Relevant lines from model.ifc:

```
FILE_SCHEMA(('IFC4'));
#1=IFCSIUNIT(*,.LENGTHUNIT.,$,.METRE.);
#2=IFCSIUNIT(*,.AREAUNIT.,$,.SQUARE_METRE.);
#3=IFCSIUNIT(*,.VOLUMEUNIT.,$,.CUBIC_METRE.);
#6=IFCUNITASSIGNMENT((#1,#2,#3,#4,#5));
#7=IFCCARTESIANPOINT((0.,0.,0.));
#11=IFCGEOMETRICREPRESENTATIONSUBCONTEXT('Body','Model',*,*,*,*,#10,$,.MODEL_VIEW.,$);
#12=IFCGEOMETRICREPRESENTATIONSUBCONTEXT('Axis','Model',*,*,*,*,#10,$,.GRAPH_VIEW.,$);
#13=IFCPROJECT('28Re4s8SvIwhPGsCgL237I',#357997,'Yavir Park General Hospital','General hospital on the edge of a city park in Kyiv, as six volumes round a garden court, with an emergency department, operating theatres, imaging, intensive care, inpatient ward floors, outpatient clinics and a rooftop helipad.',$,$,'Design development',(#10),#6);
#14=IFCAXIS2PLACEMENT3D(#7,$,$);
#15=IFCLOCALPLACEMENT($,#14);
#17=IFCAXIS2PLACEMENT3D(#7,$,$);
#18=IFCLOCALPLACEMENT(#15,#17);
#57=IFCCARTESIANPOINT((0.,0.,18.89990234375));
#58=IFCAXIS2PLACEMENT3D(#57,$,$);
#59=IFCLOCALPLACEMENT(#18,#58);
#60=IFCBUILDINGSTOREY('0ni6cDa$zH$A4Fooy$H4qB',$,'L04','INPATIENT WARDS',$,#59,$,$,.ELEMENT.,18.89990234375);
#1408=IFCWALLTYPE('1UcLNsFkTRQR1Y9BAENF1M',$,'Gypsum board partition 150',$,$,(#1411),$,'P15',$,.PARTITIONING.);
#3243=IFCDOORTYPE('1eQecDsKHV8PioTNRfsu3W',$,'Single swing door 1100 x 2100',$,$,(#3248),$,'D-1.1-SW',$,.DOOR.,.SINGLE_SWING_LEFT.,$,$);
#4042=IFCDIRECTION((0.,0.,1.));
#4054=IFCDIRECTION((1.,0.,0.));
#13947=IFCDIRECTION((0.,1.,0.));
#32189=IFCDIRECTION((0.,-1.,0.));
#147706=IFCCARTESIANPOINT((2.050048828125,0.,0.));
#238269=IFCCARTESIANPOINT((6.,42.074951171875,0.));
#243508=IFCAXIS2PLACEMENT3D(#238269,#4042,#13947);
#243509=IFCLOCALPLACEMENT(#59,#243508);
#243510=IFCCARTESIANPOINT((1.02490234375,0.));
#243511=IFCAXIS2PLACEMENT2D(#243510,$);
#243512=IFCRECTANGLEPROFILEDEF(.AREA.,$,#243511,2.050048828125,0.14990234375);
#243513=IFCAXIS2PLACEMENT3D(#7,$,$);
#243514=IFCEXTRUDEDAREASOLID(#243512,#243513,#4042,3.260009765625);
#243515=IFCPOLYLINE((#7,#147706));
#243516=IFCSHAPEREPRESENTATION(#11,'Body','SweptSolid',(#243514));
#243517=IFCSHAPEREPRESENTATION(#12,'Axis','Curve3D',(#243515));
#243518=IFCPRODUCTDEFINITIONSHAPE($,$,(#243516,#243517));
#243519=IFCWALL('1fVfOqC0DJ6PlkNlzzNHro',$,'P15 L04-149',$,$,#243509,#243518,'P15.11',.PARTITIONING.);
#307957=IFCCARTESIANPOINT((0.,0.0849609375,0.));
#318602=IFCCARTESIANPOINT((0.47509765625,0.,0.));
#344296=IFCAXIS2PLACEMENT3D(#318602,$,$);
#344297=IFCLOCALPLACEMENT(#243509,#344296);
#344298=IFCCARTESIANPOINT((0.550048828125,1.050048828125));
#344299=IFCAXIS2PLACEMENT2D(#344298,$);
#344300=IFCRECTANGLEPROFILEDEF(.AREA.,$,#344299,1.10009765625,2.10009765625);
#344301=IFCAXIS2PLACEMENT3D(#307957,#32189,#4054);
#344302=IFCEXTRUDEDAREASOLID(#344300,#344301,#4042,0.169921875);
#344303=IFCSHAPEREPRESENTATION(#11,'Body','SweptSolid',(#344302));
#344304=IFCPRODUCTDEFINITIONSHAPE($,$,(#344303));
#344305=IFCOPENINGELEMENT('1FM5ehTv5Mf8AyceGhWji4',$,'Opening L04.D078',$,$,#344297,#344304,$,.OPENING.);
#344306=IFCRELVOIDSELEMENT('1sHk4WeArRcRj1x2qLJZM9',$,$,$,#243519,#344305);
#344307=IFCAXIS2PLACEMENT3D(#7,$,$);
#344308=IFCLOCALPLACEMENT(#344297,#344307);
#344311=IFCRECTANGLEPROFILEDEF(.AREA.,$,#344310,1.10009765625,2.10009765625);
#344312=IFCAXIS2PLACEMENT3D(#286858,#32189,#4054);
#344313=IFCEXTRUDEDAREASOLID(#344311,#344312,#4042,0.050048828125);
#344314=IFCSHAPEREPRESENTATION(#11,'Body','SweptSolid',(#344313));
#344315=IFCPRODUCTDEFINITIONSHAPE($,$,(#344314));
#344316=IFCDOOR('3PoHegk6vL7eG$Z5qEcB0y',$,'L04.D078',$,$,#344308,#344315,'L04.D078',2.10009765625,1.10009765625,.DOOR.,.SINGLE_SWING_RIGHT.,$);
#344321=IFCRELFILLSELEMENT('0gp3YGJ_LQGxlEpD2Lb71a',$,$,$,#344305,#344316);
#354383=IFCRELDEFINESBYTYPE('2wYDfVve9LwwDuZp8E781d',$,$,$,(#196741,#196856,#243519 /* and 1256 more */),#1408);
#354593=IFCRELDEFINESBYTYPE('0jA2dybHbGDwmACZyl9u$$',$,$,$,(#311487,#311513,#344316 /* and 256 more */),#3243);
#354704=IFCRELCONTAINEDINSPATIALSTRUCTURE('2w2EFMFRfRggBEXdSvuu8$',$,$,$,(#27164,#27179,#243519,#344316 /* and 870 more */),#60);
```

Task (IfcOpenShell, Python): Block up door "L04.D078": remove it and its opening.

```python
import ifcopenshell
import ifcopenshell.api.feature
import ifcopenshell.api.root
import ifcopenshell.geom
import ifcopenshell.util.shape

model = ifcopenshell.open("model.ifc")
settings = ifcopenshell.geom.settings()


def volume(element):
    """Net volume in cubic metres, openings subtracted."""
    shape = ifcopenshell.geom.create_shape(settings, element)
    return ifcopenshell.util.shape.get_volume(shape.geometry)


door = model.by_guid("3PoHegk6vL7eG$Z5qEcB0y")
opening = door.FillsVoids[0].RelatingOpeningElement
wall = opening.VoidsElements[0].RelatingBuildingElement
before = volume(wall)

ifcopenshell.api.root.remove_product(model, product=door)
ifcopenshell.api.feature.remove_feature(model, feature=opening)

after = volume(wall)

print(f"wall volume {before:.3f} -> {after:.3f} m3")

model.write("model_edited.ifc")
```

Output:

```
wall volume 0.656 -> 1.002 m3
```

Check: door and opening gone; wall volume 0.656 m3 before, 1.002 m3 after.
